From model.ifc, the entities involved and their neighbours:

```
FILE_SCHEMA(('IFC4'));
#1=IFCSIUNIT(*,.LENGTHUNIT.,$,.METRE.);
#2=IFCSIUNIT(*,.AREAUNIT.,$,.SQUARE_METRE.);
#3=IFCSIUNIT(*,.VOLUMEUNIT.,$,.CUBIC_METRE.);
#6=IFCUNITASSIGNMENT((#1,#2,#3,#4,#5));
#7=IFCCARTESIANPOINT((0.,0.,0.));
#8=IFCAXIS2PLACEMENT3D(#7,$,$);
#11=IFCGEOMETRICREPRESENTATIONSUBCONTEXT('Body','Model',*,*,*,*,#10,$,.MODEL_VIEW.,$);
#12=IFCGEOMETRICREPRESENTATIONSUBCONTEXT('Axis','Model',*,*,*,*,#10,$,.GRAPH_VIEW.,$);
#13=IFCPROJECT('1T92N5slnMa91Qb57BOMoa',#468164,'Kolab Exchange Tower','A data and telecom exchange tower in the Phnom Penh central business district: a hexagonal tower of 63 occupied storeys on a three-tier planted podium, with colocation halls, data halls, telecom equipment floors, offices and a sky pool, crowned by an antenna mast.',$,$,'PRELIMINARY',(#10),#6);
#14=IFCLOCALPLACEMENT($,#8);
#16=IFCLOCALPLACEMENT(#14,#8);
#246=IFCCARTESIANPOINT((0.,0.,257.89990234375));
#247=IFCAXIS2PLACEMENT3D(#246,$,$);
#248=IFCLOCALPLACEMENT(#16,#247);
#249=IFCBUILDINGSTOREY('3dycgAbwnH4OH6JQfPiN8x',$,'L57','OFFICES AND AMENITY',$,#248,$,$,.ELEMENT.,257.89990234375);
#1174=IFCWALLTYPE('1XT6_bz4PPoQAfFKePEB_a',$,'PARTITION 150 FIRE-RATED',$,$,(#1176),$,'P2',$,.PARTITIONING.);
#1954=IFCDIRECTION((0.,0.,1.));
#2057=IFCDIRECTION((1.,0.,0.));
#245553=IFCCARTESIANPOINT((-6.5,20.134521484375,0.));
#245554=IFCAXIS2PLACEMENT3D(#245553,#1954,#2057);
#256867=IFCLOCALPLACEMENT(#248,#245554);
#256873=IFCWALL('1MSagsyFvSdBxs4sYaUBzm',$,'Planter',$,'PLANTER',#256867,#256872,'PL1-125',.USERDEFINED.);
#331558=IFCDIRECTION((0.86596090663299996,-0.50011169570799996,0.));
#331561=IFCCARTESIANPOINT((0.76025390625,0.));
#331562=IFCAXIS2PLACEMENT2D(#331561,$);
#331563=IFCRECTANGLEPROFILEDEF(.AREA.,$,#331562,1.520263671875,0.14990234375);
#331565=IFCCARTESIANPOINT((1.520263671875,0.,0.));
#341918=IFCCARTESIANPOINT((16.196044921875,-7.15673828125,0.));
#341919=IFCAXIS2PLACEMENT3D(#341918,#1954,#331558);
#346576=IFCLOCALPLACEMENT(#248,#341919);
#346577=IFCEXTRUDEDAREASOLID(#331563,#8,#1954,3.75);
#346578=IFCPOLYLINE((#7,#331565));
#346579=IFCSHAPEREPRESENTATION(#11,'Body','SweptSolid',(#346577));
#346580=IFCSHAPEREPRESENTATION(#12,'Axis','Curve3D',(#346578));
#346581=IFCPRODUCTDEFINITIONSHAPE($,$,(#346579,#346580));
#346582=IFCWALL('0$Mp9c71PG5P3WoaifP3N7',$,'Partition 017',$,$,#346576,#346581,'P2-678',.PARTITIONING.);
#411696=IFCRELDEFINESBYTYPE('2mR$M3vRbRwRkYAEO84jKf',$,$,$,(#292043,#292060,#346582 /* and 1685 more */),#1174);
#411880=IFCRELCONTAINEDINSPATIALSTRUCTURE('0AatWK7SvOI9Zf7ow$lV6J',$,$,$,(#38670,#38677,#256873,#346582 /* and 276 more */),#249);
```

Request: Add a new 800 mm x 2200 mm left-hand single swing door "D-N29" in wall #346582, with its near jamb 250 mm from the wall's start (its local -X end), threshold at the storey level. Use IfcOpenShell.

```python
import numpy as np
import ifcopenshell
import ifcopenshell.api.feature
import ifcopenshell.api.geometry
import ifcopenshell.api.root
import ifcopenshell.api.spatial
import ifcopenshell.geom
import ifcopenshell.util.element
import ifcopenshell.util.placement
import ifcopenshell.util.representation
import ifcopenshell.util.shape
import ifcopenshell.util.unit

model = ifcopenshell.open("model.ifc")
unit_scale = ifcopenshell.util.unit.calculate_unit_scale(model)
settings = ifcopenshell.geom.settings()


def volume(element):
    """Net volume in cubic metres, openings subtracted."""
    shape = ifcopenshell.geom.create_shape(settings, element)
    return ifcopenshell.util.shape.get_volume(shape.geometry)


wall = model.by_guid("0$Mp9c71PG5P3WoaifP3N7")
storey = ifcopenshell.util.element.get_container(wall, ifc_class="IfcBuildingStorey")
context = ifcopenshell.util.representation.get_context(model, "Model", "Body", "MODEL_VIEW")
before = volume(wall)

width, height, from_end, sill = 0.8, 2.2, 0.25, 0.0  # metres

# The wall runs along its own X axis, and the end named is its -X end.
wall_shape = ifcopenshell.geom.create_shape(settings, wall)
x, y, z = ifcopenshell.util.shape.get_vertices(wall_shape.geometry).T
start = x.min() + from_end
face, thickness = float(y.min()), float(y.max() - y.min())
wall_matrix = ifcopenshell.util.placement.get_local_placement(wall.ObjectPlacement)
level = ifcopenshell.util.placement.get_local_placement(storey.ObjectPlacement)[2, 3]


def in_wall(x, y):
    """Placement at x, y metres in the wall's axes, at sill height."""
    matrix = wall_matrix.copy()
    matrix[:, 3] = wall_matrix @ np.array([x / unit_scale, y / unit_scale, 0.0, 1.0])
    matrix[2, 3] = level + sill / unit_scale
    return matrix


# Opening: a box that overshoots both wall faces by 50 mm.
opening = ifcopenshell.api.root.create_entity(model, ifc_class="IfcOpeningElement", predefined_type="OPENING")
box = ifcopenshell.api.geometry.add_wall_representation(
    model, context=context, length=width, height=height, thickness=thickness + 0.1
)
ifcopenshell.api.geometry.assign_representation(model, product=opening, representation=box)
ifcopenshell.api.geometry.edit_object_placement(model, product=opening, matrix=in_wall(start, face - 0.05), is_si=False)
ifcopenshell.api.feature.add_feature(model, feature=opening, element=wall)

door = ifcopenshell.api.root.create_entity(model, ifc_class="IfcDoor", name="D-N29", predefined_type="DOOR")
door.OverallWidth, door.OverallHeight = width / unit_scale, height / unit_scale
door.OperationType = "SINGLE_SWING_LEFT"
body = ifcopenshell.api.geometry.add_door_representation(
    model,
    context=context,
    overall_width=door.OverallWidth,
    overall_height=door.OverallHeight,
    operation_type="SINGLE_SWING_LEFT",
    lining_properties={"LiningDepth": thickness / unit_scale, "ThresholdDepth": thickness / unit_scale},
)
ifcopenshell.api.geometry.assign_representation(model, product=door, representation=body)
ifcopenshell.api.spatial.assign_container(model, products=[door], relating_structure=storey)
ifcopenshell.api.feature.add_filling(model, opening=opening, element=door)

# The lining spans the wall, so the door starts at the wall face.
ifcopenshell.api.geometry.edit_object_placement(model, product=door, matrix=in_wall(start, face), is_si=False)

after = volume(wall)

print(f"wall volume {before:.3f} -> {after:.3f} m3")

model.write("model_v2.ifc")
```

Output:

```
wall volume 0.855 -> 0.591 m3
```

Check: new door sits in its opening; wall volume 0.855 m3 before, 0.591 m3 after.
